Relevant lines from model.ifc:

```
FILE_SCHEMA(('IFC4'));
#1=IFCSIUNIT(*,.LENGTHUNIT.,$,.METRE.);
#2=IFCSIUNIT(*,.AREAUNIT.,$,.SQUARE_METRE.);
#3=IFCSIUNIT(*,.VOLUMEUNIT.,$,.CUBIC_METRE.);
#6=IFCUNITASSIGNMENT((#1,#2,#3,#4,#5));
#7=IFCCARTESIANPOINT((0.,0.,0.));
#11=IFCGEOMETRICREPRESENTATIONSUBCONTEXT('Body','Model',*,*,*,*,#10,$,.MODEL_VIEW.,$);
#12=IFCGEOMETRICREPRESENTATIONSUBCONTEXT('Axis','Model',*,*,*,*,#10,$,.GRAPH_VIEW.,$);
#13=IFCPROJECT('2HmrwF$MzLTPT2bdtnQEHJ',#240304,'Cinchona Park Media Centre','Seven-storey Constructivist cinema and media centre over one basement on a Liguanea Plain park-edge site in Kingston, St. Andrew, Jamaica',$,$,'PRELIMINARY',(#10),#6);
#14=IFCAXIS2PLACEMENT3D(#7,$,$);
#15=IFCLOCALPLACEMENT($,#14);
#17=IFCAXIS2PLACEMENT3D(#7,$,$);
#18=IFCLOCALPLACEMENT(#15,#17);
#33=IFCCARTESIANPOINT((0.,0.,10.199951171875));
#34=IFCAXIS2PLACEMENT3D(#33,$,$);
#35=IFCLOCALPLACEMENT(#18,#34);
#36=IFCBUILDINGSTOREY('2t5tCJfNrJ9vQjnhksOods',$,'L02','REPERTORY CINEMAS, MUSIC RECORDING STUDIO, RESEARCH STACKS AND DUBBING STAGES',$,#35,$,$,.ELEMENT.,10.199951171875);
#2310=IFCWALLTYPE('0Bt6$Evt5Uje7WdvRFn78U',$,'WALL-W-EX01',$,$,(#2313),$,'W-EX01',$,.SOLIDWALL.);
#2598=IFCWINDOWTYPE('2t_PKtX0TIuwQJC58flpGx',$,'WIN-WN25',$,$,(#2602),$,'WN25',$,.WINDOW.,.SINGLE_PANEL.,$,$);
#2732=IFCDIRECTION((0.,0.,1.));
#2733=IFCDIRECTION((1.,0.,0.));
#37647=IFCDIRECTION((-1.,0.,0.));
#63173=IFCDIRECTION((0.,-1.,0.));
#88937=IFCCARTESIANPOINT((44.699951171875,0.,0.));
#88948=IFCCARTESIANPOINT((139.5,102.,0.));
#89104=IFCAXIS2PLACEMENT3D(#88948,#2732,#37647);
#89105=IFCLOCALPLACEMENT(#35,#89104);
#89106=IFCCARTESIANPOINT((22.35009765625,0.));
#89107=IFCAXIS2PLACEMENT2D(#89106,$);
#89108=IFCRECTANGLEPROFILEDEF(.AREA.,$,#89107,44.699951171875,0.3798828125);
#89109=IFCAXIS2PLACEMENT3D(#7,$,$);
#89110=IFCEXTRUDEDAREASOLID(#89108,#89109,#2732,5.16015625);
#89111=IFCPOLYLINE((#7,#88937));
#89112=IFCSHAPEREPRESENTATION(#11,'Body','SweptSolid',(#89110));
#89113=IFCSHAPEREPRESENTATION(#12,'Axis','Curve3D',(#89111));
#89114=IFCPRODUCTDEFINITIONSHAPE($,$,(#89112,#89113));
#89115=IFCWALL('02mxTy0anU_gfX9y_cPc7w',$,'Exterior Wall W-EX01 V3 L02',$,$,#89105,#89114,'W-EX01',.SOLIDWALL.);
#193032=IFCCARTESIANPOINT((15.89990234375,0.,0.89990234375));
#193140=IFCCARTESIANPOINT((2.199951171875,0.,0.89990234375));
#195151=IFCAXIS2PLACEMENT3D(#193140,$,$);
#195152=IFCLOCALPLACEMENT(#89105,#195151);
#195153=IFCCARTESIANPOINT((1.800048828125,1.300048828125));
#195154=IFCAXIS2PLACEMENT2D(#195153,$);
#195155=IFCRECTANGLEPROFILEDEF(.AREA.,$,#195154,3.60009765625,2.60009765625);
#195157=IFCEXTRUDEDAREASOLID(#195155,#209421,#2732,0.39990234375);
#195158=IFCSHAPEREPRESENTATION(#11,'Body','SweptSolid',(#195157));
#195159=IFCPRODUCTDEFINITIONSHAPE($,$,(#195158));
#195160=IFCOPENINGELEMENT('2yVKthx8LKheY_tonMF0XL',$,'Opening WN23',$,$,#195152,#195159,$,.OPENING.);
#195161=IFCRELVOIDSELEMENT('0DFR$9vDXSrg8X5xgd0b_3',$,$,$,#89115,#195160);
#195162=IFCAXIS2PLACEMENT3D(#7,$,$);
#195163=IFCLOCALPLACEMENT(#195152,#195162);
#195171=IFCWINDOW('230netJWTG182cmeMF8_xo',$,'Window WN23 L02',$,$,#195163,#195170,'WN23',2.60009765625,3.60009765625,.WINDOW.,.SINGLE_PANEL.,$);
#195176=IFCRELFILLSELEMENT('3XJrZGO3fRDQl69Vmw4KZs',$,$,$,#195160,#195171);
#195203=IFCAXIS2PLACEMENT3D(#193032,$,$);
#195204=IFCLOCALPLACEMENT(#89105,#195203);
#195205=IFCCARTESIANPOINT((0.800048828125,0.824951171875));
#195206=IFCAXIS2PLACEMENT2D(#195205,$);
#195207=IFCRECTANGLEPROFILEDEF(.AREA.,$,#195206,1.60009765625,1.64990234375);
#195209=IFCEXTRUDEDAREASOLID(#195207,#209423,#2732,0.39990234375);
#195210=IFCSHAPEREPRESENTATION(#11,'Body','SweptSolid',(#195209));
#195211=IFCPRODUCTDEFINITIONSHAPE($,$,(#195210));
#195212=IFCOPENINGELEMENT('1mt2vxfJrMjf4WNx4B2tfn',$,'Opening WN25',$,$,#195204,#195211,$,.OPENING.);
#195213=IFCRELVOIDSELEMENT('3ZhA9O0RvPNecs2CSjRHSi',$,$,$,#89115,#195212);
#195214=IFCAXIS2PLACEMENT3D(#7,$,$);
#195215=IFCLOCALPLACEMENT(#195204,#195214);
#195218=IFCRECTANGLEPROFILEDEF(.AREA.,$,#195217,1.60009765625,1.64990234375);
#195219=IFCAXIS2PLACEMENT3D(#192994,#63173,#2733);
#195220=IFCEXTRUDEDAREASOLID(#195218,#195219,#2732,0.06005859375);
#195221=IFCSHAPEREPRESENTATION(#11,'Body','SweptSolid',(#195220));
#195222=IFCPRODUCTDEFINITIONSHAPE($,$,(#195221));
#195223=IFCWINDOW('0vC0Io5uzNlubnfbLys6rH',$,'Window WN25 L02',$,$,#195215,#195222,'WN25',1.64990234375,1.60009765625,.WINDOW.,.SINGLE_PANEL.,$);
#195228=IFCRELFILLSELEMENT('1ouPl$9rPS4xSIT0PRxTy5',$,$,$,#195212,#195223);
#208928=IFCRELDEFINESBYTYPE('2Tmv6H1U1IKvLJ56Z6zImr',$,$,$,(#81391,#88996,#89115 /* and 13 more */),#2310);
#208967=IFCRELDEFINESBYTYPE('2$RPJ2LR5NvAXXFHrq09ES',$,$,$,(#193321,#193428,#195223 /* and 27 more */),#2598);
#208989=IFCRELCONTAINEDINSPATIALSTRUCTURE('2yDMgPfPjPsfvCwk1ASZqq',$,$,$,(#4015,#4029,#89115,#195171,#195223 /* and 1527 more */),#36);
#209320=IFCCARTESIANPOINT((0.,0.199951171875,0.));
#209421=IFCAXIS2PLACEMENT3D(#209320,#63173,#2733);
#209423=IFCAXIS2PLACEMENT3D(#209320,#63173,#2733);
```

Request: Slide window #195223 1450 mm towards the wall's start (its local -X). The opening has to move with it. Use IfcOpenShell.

```python
import ifcopenshell
import ifcopenshell.api.geometry
import ifcopenshell.util.placement
import ifcopenshell.util.unit

model = ifcopenshell.open("model.ifc")
unit_scale = ifcopenshell.util.unit.calculate_unit_scale(model)

window = model.by_guid("0vC0Io5uzNlubnfbLys6rH")
opening = window.FillsVoids[0].RelatingOpeningElement
wall = opening.VoidsElements[0].RelatingBuildingElement

wall_matrix = ifcopenshell.util.placement.get_local_placement(wall.ObjectPlacement)
shift = wall_matrix[:3, 0] * -1.45 / unit_scale
before = ifcopenshell.util.placement.get_local_placement(window.ObjectPlacement)[:3, 3].copy()

# The window is placed relative to its opening, so it follows when the opening moves.
matrix = ifcopenshell.util.placement.get_local_placement(opening.ObjectPlacement)
matrix[:3, 3] += shift
ifcopenshell.api.geometry.edit_object_placement(
    model, product=opening, matrix=matrix, is_si=False, should_transform_children=True
)

after = ifcopenshell.util.placement.get_local_placement(window.ObjectPlacement)[:3, 3]
print("window moved by", (after - before).round(3) + 0.0)

model.write("model_v2.ifc")
```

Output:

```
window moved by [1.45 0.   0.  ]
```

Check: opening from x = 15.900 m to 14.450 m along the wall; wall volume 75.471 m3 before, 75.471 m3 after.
